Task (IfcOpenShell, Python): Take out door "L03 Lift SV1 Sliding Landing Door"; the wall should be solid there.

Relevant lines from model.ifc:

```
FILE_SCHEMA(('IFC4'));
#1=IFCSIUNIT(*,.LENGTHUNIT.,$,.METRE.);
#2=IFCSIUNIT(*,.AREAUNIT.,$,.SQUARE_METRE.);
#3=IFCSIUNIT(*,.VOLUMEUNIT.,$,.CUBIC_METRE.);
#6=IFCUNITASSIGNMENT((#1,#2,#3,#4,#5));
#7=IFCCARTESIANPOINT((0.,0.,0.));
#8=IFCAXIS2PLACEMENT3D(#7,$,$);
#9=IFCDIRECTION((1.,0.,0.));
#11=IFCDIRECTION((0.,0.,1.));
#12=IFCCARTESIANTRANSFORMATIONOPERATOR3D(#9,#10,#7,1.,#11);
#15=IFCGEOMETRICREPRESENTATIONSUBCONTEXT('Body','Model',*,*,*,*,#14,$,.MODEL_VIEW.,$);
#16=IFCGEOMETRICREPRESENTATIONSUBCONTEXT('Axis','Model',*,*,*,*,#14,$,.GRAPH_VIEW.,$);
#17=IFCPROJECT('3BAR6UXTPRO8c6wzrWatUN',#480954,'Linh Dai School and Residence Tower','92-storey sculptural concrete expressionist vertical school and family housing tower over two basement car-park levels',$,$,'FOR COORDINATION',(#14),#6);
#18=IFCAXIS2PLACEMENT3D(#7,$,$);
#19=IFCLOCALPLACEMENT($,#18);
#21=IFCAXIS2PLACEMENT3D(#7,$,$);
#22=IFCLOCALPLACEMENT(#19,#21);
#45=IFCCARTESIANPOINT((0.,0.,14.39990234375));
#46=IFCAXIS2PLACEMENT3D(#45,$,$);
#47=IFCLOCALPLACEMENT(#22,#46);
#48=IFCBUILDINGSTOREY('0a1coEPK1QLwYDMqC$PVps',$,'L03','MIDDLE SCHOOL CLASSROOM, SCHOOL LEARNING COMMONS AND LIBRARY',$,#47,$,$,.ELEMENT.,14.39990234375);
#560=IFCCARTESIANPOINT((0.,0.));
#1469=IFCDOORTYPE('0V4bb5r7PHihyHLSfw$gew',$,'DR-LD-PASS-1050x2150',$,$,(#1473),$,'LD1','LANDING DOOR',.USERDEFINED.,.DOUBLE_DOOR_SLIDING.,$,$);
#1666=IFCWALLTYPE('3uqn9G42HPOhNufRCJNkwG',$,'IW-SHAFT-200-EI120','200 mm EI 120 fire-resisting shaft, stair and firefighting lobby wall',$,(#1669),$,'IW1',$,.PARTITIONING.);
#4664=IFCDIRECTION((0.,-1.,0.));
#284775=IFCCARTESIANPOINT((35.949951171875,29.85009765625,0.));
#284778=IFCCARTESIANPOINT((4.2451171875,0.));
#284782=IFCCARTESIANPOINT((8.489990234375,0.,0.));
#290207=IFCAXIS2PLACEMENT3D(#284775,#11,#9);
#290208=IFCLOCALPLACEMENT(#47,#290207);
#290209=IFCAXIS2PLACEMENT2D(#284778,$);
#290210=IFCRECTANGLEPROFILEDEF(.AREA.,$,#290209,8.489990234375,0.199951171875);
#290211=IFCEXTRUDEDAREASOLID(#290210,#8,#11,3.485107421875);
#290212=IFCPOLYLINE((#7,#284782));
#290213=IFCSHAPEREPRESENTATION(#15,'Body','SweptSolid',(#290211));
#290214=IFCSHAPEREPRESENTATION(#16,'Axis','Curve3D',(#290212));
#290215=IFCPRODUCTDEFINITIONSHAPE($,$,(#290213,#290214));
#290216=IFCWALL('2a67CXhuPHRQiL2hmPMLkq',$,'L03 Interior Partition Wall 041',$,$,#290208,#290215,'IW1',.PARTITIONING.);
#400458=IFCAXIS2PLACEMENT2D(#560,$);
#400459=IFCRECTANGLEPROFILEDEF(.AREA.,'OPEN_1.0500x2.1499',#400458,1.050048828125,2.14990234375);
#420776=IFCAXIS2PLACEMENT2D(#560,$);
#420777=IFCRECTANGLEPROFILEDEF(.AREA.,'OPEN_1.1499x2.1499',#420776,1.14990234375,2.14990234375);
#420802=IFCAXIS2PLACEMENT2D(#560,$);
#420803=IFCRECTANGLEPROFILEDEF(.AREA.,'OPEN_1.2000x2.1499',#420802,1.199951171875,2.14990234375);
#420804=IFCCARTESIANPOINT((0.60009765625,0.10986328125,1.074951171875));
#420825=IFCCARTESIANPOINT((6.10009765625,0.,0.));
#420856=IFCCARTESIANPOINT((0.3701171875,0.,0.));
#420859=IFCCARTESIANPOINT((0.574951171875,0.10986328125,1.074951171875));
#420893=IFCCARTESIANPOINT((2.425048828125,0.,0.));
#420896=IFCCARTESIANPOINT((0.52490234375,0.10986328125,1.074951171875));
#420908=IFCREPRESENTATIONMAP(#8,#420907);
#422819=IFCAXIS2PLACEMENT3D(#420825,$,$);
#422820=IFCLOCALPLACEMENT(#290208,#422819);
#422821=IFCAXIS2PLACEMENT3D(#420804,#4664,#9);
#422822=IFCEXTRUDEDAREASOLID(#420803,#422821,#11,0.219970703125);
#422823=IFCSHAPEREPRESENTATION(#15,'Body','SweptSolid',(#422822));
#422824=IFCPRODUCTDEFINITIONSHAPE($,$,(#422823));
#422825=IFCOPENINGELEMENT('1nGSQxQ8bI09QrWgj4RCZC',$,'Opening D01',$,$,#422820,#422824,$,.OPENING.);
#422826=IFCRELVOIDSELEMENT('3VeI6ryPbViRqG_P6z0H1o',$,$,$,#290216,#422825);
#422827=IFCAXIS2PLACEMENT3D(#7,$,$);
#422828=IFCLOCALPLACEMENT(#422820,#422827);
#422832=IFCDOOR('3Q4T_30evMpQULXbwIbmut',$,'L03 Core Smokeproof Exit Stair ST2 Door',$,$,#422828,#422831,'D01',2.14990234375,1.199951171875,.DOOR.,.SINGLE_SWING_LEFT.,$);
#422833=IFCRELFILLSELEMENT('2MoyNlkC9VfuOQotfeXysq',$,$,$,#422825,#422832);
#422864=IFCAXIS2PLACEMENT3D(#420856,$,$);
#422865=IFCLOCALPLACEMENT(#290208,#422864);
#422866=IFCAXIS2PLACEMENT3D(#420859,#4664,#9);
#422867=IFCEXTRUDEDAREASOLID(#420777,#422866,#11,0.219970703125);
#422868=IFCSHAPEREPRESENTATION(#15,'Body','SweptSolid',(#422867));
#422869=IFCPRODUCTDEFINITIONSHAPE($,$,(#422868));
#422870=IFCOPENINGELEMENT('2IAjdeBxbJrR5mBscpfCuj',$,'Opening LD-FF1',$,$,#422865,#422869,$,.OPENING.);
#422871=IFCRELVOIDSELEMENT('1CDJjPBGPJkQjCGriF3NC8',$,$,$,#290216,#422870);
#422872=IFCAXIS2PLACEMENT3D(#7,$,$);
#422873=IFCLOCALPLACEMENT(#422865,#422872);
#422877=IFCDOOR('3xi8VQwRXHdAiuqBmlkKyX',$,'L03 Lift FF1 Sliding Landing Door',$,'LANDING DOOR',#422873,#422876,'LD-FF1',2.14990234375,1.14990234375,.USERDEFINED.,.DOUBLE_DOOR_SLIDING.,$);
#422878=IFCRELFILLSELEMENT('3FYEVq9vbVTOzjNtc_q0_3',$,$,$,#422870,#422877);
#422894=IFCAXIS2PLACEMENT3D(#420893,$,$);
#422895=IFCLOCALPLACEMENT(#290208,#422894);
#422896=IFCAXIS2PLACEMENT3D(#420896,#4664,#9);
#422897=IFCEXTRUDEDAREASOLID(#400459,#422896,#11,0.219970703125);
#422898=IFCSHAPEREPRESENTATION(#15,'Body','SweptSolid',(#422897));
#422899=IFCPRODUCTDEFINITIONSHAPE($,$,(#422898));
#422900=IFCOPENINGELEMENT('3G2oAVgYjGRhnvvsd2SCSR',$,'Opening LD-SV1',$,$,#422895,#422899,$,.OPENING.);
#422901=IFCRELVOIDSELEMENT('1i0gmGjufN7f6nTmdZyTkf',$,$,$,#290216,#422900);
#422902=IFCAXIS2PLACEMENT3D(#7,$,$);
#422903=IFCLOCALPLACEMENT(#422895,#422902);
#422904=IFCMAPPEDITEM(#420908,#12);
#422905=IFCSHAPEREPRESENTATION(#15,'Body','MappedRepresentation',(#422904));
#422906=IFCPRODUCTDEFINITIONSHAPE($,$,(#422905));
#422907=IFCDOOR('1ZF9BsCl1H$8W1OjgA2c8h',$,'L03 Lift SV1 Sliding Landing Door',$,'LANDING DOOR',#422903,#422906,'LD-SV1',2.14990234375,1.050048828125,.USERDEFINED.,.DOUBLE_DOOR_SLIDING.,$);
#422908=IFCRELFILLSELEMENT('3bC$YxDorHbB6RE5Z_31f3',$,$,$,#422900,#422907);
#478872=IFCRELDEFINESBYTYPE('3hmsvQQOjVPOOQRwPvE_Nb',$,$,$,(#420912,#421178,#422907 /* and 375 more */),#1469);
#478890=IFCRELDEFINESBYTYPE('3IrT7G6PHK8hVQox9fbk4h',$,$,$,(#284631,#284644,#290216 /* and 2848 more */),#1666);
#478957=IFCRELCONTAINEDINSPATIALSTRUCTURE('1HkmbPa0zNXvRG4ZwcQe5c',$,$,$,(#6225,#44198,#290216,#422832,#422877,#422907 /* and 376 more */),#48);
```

```python
import ifcopenshell
import ifcopenshell.api.feature
import ifcopenshell.api.root
import ifcopenshell.geom
import ifcopenshell.util.shape

model = ifcopenshell.open("model.ifc")
settings = ifcopenshell.geom.settings()


def volume(element):
    """Net volume in cubic metres, openings subtracted."""
    shape = ifcopenshell.geom.create_shape(settings, element)
    return ifcopenshell.util.shape.get_volume(shape.geometry)


door = model.by_guid("1ZF9BsCl1H$8W1OjgA2c8h")
opening = door.FillsVoids[0].RelatingOpeningElement
wall = opening.VoidsElements[0].RelatingBuildingElement
before = volume(wall)

ifcopenshell.api.root.remove_product(model, product=door)
ifcopenshell.api.feature.remove_feature(model, feature=opening)

after = volume(wall)

print(f"wall volume {before:.3f} -> {after:.3f} m3")

model.write("model-out.ifc")
```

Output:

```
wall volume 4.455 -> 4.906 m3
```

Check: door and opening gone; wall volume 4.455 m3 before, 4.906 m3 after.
